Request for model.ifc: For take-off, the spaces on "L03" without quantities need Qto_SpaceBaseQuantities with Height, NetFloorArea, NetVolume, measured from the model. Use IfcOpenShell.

First a look at what the model holds.

```python
import ifcopenshell
import ifcopenshell.util.element
import ifcopenshell.util.unit

model = ifcopenshell.open("model.ifc")
print(model.schema)
for unit_type in ("LENGTHUNIT", "AREAUNIT", "VOLUMEUNIT"):
    print(unit_type, ifcopenshell.util.unit.calculate_unit_scale(model, unit_type))
storey = next(s for s in model.by_type("IfcBuildingStorey") if s.Name == "L03")
spaces = [e for e in ifcopenshell.util.element.get_decomposition(storey) if e.is_a("IfcSpace")]
for e in sorted(spaces, key=lambda e: e.id()):
    print(e.id(), e.is_a(), e.Name, list(ifcopenshell.util.element.get_psets(e, qtos_only=True)), sep=" | ")
```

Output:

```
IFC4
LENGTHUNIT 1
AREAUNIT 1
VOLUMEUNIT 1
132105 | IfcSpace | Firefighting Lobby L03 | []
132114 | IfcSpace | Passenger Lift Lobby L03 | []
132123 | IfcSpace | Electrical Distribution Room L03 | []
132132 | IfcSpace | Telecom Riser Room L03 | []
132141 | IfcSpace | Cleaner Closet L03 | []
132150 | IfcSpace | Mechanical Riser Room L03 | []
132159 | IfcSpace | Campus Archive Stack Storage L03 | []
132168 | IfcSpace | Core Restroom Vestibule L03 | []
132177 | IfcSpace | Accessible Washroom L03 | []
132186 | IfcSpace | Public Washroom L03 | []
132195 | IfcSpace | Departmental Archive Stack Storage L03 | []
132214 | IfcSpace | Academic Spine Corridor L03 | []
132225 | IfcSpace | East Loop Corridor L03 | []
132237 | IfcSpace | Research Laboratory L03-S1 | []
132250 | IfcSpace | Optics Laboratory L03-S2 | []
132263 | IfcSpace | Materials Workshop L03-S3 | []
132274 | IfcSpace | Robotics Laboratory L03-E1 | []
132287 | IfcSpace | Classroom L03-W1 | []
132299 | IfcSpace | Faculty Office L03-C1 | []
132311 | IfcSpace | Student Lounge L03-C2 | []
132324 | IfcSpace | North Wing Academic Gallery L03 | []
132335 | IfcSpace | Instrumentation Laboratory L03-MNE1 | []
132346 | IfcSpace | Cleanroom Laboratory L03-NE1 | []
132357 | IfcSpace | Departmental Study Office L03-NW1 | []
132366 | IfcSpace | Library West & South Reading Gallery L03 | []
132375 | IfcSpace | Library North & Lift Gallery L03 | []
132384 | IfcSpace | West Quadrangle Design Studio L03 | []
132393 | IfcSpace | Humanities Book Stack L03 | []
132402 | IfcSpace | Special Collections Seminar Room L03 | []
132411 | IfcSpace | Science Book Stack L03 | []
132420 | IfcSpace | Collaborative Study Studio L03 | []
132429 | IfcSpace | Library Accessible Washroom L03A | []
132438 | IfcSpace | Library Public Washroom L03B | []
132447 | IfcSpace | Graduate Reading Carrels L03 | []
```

```python
import ifcopenshell
import ifcopenshell.api.pset
import ifcopenshell.geom
import ifcopenshell.util.element
import ifcopenshell.util.shape
import ifcopenshell.util.unit

model = ifcopenshell.open("model.ifc")
unit_scale = ifcopenshell.util.unit.calculate_unit_scale(model)
area_scale = ifcopenshell.util.unit.calculate_unit_scale(model, "AREAUNIT")
volume_scale = ifcopenshell.util.unit.calculate_unit_scale(model, "VOLUMEUNIT")
settings = ifcopenshell.geom.settings()

storey = next(s for s in model.by_type("IfcBuildingStorey") if s.Name == "L03")
spaces = [e for e in ifcopenshell.util.element.get_decomposition(storey) if e.is_a("IfcSpace")]

for e in sorted(spaces, key=lambda e: e.id()):
    if ifcopenshell.util.element.get_psets(e, qtos_only=True, should_inherit=False):
        continue
    # Geometry comes back in metres, in the element's own axes.
    shape = ifcopenshell.geom.create_shape(settings, e)
    values = {
        "Height": ifcopenshell.util.shape.get_z(shape.geometry) / unit_scale,
        "NetFloorArea": ifcopenshell.util.shape.get_footprint_area(shape.geometry) / area_scale,
        "NetVolume": ifcopenshell.util.shape.get_volume(shape.geometry) / volume_scale,
    }
    qto = ifcopenshell.api.pset.add_qto(model, product=e, name="Qto_SpaceBaseQuantities")
    ifcopenshell.api.pset.edit_qto(model, qto=qto, properties=values)
    print(e.id(), {k: round(v, 3) for k, v in values.items()})

model.write("model_edited.ifc")
```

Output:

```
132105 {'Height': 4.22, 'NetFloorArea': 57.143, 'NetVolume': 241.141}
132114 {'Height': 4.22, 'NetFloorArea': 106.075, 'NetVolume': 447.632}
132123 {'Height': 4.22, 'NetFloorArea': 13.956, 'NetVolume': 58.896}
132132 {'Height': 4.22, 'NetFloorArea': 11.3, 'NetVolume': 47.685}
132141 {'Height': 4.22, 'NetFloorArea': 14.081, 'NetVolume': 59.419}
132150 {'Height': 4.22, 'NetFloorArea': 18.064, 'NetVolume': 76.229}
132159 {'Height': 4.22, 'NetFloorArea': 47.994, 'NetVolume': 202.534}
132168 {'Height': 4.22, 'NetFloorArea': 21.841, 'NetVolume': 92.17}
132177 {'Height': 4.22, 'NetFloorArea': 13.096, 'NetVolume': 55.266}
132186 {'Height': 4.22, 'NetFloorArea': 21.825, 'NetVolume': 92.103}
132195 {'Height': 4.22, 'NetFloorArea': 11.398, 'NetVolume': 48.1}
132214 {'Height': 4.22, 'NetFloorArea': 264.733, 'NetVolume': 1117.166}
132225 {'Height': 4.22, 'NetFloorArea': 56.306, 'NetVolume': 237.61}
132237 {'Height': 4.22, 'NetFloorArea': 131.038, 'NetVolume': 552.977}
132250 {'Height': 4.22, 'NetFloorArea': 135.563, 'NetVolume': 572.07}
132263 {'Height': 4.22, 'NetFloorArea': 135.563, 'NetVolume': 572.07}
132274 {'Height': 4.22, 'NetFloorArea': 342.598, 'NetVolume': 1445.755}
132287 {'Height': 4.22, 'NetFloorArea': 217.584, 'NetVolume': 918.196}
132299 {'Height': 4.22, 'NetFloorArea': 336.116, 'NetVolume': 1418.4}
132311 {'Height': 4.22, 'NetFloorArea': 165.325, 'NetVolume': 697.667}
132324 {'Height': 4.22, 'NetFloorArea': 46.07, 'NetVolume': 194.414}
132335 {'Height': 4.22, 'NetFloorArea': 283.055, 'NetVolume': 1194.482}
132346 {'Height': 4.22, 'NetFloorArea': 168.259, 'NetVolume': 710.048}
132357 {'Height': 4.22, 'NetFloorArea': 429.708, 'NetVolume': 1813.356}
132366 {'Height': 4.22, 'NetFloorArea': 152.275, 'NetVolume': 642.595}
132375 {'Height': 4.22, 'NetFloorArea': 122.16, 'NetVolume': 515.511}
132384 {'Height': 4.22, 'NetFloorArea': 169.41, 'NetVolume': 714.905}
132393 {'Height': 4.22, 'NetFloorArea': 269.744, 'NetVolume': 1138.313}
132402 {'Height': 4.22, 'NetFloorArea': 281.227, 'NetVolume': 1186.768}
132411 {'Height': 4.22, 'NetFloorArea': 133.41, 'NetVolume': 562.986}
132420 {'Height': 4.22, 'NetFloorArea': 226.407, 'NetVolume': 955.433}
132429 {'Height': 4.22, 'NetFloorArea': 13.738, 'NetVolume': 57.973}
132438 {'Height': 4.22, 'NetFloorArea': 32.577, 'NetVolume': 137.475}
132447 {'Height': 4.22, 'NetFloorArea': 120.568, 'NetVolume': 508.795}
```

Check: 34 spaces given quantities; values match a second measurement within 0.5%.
